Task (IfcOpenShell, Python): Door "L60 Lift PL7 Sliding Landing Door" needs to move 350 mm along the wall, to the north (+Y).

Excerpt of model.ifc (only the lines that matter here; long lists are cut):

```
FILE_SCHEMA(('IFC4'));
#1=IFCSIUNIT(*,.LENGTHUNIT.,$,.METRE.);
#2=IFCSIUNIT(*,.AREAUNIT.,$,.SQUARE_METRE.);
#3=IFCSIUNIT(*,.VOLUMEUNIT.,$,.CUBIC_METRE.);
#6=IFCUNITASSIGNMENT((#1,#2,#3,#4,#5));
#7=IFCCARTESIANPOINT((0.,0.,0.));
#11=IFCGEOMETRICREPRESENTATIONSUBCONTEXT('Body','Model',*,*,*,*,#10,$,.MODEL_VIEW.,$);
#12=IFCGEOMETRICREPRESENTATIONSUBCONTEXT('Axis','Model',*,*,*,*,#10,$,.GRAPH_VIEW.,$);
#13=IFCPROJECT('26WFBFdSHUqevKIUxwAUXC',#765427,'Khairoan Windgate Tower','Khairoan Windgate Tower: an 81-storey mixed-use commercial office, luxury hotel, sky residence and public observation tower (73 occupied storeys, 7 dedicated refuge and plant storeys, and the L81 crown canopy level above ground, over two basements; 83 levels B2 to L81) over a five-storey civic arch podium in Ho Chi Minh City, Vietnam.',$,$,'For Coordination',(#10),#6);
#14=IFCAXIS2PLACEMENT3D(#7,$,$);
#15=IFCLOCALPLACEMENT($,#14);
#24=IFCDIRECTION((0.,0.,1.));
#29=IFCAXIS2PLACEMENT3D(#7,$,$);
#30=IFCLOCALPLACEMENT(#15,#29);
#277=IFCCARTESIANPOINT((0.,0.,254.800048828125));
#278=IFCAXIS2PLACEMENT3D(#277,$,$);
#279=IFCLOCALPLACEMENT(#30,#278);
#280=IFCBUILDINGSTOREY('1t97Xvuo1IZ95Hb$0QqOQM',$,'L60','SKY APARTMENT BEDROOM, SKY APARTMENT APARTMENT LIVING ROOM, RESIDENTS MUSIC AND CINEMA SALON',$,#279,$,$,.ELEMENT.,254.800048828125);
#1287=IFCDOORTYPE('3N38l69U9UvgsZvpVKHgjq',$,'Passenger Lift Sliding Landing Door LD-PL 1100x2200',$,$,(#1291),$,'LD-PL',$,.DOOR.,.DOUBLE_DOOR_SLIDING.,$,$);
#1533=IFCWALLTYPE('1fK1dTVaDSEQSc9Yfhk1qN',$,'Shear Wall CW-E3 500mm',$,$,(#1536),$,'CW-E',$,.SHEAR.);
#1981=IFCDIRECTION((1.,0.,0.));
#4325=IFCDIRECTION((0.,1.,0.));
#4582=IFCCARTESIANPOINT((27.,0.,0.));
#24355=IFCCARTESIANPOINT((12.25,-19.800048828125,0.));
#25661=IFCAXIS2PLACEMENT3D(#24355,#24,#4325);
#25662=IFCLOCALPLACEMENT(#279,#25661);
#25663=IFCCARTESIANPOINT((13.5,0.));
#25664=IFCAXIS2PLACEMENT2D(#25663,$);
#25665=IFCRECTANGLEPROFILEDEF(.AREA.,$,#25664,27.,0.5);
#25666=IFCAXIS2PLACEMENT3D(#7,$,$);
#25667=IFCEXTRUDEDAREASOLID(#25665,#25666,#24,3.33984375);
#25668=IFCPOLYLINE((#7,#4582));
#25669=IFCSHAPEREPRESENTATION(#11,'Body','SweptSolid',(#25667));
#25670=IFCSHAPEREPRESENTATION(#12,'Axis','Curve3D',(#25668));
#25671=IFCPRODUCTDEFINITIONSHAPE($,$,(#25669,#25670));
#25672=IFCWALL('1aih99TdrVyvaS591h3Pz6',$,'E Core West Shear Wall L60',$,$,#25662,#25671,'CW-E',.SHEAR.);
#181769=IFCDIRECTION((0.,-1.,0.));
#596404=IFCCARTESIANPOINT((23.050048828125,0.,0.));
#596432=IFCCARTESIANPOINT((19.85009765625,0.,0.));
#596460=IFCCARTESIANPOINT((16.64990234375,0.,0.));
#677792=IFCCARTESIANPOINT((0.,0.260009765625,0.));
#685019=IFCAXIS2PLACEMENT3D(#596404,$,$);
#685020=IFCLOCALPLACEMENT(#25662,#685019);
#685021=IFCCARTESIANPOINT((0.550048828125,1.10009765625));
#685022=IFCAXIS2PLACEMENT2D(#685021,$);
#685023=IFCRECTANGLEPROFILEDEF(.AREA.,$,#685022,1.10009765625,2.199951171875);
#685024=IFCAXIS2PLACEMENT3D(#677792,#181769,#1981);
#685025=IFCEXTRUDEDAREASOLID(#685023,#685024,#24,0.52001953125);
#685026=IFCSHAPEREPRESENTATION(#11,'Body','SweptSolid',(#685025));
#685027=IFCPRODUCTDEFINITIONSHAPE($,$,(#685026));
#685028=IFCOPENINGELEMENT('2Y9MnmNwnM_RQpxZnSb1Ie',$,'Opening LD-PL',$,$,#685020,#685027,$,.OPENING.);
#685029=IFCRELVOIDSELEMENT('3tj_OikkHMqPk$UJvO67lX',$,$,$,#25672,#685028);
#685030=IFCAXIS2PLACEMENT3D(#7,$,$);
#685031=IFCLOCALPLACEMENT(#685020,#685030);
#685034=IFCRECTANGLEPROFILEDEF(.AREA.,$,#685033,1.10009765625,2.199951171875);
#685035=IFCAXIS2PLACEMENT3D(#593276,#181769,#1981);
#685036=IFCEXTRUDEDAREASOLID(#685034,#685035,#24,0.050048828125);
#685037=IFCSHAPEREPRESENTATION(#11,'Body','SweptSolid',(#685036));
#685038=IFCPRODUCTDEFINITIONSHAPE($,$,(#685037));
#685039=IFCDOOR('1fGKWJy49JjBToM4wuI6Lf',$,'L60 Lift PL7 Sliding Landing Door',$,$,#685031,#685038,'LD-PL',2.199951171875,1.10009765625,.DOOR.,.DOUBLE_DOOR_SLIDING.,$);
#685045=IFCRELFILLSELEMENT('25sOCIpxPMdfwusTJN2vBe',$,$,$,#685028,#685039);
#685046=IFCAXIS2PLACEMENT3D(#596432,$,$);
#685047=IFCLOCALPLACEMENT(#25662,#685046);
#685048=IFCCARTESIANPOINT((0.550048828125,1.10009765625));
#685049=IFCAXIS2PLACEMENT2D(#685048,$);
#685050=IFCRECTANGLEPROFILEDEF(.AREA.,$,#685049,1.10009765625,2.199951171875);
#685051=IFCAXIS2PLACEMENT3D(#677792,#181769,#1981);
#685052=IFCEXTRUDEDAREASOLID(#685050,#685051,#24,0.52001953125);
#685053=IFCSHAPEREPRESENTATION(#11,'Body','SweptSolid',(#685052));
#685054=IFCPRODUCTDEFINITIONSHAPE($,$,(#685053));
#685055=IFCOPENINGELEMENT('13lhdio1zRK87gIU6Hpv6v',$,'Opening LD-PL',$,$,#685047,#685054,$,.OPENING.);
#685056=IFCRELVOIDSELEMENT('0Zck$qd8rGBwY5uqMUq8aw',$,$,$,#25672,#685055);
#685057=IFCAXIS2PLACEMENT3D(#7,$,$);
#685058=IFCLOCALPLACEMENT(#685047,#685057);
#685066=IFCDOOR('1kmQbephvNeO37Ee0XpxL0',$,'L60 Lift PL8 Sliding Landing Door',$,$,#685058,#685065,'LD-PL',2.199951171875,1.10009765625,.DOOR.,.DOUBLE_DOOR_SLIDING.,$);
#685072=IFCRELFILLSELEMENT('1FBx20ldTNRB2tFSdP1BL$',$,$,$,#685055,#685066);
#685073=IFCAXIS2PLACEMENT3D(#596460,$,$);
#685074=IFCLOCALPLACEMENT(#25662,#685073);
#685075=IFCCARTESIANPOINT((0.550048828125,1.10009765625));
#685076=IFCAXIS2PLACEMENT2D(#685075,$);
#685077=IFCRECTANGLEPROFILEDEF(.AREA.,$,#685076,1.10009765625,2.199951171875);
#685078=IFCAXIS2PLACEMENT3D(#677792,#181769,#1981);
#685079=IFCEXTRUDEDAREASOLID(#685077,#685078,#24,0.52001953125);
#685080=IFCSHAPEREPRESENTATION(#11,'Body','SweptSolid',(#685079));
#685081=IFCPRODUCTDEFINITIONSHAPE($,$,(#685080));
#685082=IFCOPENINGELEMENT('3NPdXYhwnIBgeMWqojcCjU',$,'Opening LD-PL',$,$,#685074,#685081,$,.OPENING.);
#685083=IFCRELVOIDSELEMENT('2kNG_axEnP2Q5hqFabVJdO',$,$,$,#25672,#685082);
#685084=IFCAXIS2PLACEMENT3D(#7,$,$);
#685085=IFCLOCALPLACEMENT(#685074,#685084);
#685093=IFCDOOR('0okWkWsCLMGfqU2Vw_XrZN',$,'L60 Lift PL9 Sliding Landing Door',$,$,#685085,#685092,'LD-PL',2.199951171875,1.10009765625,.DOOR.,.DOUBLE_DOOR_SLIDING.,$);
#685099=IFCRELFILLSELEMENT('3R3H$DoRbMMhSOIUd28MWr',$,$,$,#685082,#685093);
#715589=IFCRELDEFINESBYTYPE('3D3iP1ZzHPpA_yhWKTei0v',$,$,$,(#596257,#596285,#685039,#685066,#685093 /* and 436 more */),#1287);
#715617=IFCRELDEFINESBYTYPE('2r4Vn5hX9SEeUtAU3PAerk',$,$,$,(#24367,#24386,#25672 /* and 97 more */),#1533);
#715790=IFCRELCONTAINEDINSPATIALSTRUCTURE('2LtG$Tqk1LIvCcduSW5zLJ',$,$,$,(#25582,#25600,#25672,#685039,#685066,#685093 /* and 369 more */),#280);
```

```python
import ifcopenshell
import ifcopenshell.api.geometry
import ifcopenshell.util.placement
import ifcopenshell.util.unit

model = ifcopenshell.open("model.ifc")
unit_scale = ifcopenshell.util.unit.calculate_unit_scale(model)

door = model.by_guid("1fGKWJy49JjBToM4wuI6Lf")
opening = door.FillsVoids[0].RelatingOpeningElement
wall = opening.VoidsElements[0].RelatingBuildingElement

wall_matrix = ifcopenshell.util.placement.get_local_placement(wall.ObjectPlacement)
shift = wall_matrix[:3, 0] * 0.35 / unit_scale
before = ifcopenshell.util.placement.get_local_placement(door.ObjectPlacement)[:3, 3].copy()

# The door is placed relative to its opening, so it follows when the opening moves.
matrix = ifcopenshell.util.placement.get_local_placement(opening.ObjectPlacement)
matrix[:3, 3] += shift
ifcopenshell.api.geometry.edit_object_placement(
    model, product=opening, matrix=matrix, is_si=False, should_transform_children=True
)

after = ifcopenshell.util.placement.get_local_placement(door.ObjectPlacement)[:3, 3]
print("door moved by", (after - before).round(3) + 0.0)

model.write("model_v2.ifc")
```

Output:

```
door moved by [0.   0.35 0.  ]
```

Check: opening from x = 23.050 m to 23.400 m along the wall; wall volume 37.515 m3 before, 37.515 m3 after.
